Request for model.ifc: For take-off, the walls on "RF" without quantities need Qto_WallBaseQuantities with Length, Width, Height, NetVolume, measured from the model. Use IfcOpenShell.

First a look at what the model holds.

```python
import ifcopenshell
import ifcopenshell.util.element
import ifcopenshell.util.unit

model = ifcopenshell.open("model.ifc")
print(model.schema)
for unit_type in ("LENGTHUNIT", "AREAUNIT", "VOLUMEUNIT"):
    print(unit_type, ifcopenshell.util.unit.calculate_unit_scale(model, unit_type))
storey = next(s for s in model.by_type("IfcBuildingStorey") if s.Name == "RF")
walls = [e for e in ifcopenshell.util.element.get_decomposition(storey) if e.is_a("IfcWall")]
for e in sorted(walls, key=lambda e: e.id()):
    print(e.id(), e.is_a(), e.Name, list(ifcopenshell.util.element.get_psets(e, qtos_only=True)), sep=" | ")
```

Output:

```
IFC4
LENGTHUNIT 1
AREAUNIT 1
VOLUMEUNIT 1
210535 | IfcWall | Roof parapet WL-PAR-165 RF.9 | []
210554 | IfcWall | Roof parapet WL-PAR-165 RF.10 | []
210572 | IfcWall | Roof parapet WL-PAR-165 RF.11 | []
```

```python
import ifcopenshell
import ifcopenshell.api.pset
import ifcopenshell.geom
import ifcopenshell.util.element
import ifcopenshell.util.shape
import ifcopenshell.util.unit

model = ifcopenshell.open("model.ifc")
unit_scale = ifcopenshell.util.unit.calculate_unit_scale(model)
volume_scale = ifcopenshell.util.unit.calculate_unit_scale(model, "VOLUMEUNIT")
settings = ifcopenshell.geom.settings()

storey = next(s for s in model.by_type("IfcBuildingStorey") if s.Name == "RF")
walls = [e for e in ifcopenshell.util.element.get_decomposition(storey) if e.is_a("IfcWall")]

for e in sorted(walls, key=lambda e: e.id()):
    if ifcopenshell.util.element.get_psets(e, qtos_only=True, should_inherit=False):
        continue
    # Geometry comes back in metres, in the element's own axes.
    shape = ifcopenshell.geom.create_shape(settings, e)
    values = {
        "Length": ifcopenshell.util.shape.get_x(shape.geometry) / unit_scale,
        "Width": ifcopenshell.util.shape.get_y(shape.geometry) / unit_scale,
        "Height": ifcopenshell.util.shape.get_z(shape.geometry) / unit_scale,
        "NetVolume": ifcopenshell.util.shape.get_volume(shape.geometry) / volume_scale,
    }
    qto = ifcopenshell.api.pset.add_qto(model, product=e, name="Qto_WallBaseQuantities")
    ifcopenshell.api.pset.edit_qto(model, qto=qto, properties=values)
    print(e.id(), {k: round(v, 3) for k, v in values.items()})

model.write("model_updated.ifc")
```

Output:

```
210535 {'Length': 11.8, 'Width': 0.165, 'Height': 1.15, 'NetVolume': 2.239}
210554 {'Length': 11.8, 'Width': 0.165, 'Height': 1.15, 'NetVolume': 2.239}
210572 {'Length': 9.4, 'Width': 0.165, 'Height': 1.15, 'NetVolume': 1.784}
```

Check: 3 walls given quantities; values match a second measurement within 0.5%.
